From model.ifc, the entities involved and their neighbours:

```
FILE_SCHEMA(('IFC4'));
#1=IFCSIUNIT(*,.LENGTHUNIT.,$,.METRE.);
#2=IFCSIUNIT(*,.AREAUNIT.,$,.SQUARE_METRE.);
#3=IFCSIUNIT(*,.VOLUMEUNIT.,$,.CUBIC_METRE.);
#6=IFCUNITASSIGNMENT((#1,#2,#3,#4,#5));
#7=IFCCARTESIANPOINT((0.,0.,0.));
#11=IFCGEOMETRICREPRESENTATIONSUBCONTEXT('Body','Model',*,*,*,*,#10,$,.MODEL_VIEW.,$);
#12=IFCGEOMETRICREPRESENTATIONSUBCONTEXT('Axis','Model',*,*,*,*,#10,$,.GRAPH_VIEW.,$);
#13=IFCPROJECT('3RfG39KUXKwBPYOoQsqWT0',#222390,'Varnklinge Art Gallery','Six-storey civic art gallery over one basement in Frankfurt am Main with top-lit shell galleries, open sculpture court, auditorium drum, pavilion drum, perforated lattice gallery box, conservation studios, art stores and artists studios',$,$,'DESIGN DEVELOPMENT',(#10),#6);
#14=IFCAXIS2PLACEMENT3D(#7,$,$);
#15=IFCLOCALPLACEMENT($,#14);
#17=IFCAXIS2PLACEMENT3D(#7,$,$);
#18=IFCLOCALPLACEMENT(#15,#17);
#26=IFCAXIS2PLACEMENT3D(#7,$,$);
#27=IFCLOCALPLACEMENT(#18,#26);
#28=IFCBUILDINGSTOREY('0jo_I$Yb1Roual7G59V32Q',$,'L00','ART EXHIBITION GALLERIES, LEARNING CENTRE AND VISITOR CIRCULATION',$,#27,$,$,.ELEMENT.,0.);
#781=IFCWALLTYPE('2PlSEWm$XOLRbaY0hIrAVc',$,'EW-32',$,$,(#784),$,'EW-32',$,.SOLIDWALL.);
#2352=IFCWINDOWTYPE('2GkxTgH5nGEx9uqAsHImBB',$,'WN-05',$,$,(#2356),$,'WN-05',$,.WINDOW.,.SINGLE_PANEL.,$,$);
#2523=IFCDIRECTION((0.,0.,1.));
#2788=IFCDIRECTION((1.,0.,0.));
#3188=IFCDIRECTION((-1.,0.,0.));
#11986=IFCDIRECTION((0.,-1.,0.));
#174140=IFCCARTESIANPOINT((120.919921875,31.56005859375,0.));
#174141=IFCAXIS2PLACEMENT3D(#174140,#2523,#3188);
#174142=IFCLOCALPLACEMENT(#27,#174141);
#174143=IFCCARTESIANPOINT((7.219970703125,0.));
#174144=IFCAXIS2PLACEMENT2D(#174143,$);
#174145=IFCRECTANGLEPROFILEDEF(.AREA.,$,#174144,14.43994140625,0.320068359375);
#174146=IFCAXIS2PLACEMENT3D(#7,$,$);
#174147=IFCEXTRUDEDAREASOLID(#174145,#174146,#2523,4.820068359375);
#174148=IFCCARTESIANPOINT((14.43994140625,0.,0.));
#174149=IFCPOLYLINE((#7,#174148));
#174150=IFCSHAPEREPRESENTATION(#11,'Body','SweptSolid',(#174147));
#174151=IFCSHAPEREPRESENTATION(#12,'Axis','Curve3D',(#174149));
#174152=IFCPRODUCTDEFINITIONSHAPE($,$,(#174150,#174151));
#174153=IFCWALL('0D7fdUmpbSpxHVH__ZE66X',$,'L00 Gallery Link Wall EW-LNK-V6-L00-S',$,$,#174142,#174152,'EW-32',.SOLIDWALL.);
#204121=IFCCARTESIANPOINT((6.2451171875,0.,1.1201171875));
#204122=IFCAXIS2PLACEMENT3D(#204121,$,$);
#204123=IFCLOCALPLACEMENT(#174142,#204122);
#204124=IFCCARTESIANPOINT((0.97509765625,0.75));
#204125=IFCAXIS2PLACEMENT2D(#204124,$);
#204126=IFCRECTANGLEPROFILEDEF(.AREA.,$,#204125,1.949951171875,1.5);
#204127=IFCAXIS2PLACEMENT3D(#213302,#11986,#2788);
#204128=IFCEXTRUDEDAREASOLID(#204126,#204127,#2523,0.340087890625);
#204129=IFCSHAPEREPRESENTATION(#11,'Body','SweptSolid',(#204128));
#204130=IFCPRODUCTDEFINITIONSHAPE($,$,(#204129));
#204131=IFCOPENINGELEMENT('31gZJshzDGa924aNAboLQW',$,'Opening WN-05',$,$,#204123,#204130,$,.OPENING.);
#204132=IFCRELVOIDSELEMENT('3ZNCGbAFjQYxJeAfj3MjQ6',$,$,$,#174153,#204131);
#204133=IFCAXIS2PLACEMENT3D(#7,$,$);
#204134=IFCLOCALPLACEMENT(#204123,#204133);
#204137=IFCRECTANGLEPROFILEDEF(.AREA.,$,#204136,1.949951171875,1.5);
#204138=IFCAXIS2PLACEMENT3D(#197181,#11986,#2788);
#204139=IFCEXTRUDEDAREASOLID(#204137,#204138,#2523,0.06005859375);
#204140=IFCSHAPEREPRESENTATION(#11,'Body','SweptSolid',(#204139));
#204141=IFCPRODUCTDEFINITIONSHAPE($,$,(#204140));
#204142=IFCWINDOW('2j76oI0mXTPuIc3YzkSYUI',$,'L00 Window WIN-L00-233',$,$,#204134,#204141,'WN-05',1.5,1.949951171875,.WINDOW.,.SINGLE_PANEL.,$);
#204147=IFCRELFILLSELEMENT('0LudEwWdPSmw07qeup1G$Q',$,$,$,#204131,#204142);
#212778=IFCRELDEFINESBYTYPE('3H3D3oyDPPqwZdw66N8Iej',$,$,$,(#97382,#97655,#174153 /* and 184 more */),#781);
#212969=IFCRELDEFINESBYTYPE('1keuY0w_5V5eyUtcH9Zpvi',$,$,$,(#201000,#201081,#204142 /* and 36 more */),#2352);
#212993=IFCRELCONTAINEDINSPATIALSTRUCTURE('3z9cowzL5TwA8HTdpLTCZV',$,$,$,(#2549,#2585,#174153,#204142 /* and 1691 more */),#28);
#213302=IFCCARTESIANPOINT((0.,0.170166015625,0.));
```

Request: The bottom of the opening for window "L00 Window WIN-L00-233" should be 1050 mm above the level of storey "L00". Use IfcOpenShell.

```python
import numpy as np
import ifcopenshell
import ifcopenshell.api.geometry
import ifcopenshell.geom
import ifcopenshell.util.element
import ifcopenshell.util.placement
import ifcopenshell.util.shape
import ifcopenshell.util.unit

model = ifcopenshell.open("model.ifc")
unit_scale = ifcopenshell.util.unit.calculate_unit_scale(model)

window = model.by_id(204142)
opening = window.FillsVoids[0].RelatingOpeningElement
storey = ifcopenshell.util.element.get_container(window, ifc_class="IfcBuildingStorey")
level = ifcopenshell.util.placement.get_local_placement(storey.ObjectPlacement)[2, 3]

# The opening's origin need not be at the sill, so measure its lowest point.
shape = ifcopenshell.geom.create_shape(ifcopenshell.geom.settings(), opening)
bottom = ifcopenshell.util.shape.get_shape_bottom_elevation(shape, shape.geometry) / unit_scale
dz = level + 1.05 - bottom

shift = np.array([0.0, 0.0, dz])
# The window is placed relative to its opening, so it follows when the opening moves.
matrix = ifcopenshell.util.placement.get_local_placement(opening.ObjectPlacement)
matrix[:3, 3] += shift
ifcopenshell.api.geometry.edit_object_placement(
    model, product=opening, matrix=matrix, is_si=False, should_transform_children=True
)

print(f"moved by {dz * unit_scale:+.3f} m")

model.write("model_updated.ifc")
```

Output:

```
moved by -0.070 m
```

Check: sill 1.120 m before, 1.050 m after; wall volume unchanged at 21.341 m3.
